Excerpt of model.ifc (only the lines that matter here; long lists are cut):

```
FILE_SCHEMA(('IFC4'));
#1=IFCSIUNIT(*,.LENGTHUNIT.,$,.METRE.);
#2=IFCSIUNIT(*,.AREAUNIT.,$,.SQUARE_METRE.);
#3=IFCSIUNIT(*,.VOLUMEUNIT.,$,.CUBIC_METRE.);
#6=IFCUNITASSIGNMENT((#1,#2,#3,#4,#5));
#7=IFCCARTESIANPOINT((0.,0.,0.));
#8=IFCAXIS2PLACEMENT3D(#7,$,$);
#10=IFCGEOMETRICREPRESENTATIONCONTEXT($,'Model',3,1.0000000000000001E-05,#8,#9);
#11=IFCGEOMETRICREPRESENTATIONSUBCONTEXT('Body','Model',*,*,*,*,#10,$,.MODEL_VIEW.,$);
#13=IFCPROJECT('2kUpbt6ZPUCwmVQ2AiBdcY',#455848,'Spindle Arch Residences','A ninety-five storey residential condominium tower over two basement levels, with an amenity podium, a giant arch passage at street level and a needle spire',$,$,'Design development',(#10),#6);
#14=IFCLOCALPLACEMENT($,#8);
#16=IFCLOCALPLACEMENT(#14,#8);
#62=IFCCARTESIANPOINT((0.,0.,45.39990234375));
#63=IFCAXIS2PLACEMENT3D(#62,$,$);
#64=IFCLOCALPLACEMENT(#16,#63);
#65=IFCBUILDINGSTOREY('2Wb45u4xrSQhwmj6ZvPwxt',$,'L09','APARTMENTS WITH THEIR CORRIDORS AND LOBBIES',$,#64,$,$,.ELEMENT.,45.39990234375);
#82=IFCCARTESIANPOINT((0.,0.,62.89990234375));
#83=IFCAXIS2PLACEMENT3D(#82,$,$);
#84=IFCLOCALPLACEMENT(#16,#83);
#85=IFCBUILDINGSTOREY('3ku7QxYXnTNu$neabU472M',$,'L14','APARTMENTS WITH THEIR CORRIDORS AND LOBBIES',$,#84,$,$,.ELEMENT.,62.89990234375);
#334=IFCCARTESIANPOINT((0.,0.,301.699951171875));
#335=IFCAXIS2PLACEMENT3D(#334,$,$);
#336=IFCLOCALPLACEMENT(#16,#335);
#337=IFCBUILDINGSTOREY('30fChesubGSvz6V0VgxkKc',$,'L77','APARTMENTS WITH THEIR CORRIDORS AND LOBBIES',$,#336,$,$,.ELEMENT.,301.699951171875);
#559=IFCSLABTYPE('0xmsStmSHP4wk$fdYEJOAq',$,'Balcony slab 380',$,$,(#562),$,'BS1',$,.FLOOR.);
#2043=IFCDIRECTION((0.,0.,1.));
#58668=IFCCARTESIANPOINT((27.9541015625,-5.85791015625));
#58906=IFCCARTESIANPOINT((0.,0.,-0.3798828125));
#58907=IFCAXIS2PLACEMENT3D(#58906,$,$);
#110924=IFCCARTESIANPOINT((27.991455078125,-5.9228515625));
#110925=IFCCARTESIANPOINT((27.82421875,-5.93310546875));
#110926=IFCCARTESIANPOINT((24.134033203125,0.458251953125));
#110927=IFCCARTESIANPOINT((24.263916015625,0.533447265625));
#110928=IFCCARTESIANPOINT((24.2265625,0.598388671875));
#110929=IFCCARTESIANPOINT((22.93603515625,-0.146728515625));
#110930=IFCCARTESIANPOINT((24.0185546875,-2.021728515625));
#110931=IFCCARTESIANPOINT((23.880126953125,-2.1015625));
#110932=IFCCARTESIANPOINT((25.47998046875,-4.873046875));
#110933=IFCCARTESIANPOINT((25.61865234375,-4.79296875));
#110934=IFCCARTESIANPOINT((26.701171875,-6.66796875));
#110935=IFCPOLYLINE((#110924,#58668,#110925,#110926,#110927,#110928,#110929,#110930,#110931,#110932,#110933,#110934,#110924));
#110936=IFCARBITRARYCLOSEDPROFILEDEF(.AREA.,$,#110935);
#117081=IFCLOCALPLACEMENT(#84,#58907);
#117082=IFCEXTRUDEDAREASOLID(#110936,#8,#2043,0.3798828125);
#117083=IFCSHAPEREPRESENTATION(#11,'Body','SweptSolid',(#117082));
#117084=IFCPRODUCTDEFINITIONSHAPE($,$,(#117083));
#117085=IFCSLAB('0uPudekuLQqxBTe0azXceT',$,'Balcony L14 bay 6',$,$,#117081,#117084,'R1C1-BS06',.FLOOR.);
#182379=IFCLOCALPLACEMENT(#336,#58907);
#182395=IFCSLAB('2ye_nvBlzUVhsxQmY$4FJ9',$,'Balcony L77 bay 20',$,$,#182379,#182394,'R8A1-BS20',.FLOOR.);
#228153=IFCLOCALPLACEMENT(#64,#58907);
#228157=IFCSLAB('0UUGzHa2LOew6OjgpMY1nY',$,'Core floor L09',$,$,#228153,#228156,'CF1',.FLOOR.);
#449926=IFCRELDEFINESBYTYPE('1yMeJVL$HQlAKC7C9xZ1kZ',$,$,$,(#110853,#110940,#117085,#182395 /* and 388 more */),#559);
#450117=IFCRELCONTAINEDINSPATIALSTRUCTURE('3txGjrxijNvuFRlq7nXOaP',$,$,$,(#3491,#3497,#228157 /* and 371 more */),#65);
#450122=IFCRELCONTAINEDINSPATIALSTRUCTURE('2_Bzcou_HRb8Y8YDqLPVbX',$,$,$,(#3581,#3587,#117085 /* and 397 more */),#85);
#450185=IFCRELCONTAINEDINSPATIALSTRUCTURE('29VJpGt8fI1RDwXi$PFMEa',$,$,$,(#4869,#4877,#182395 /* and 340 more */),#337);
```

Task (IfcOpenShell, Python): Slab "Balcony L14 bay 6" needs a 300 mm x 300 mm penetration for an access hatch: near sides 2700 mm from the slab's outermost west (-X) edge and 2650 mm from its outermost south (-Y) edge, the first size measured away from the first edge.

```python
import numpy as np
import ifcopenshell
import ifcopenshell.api.feature
import ifcopenshell.api.geometry
import ifcopenshell.api.root
import ifcopenshell.geom
import ifcopenshell.util.placement
import ifcopenshell.util.representation
import ifcopenshell.util.shape
import ifcopenshell.util.unit

model = ifcopenshell.open("model.ifc")
unit_scale = ifcopenshell.util.unit.calculate_unit_scale(model)
settings = ifcopenshell.geom.settings()


def volume(element):
    """Net volume in cubic metres, openings subtracted."""
    shape = ifcopenshell.geom.create_shape(settings, element)
    return ifcopenshell.util.shape.get_volume(shape.geometry)


slab = model.by_guid("0uPudekuLQqxBTe0azXceT")
before = volume(slab)

# Extent in the slab's own axes, in metres. The edges named are its -X and -Y sides.
slab_shape = ifcopenshell.geom.create_shape(settings, slab)
vertices = ifcopenshell.util.shape.get_vertices(slab_shape.geometry)
x_min, y_min, bottom = vertices.min(axis=0)
top = vertices[:, 2].max()

opening = ifcopenshell.api.root.create_entity(model, ifc_class="IfcOpeningElement", name="Access hatch opening", predefined_type="OPENING")
context = ifcopenshell.util.representation.get_context(model, "Model", "Body", "MODEL_VIEW")
width, depth = 0.3, 0.3
outline = [(0.0, 0.0), (width, 0.0), (width, depth), (0.0, depth), (0.0, 0.0)]
# Overshoot both faces by 50 mm so the cut is clean.
shape = ifcopenshell.api.geometry.add_slab_representation(
    model, context=context, depth=top - bottom + 0.1, polyline=outline
)
ifcopenshell.api.geometry.assign_representation(model, product=opening, representation=shape)

matrix = ifcopenshell.util.placement.get_local_placement(slab.ObjectPlacement)
matrix[:, 3] = matrix @ np.append(np.array([x_min + 2.7, y_min + 2.65, bottom - 0.05]) / unit_scale, 1.0)
ifcopenshell.api.geometry.edit_object_placement(model, product=opening, matrix=matrix, is_si=False)
ifcopenshell.api.feature.add_feature(model, feature=opening, element=slab)

after = volume(slab)

print(f"slab volume {before:.3f} -> {after:.3f} m3")

model.write("model_updated.ifc")
```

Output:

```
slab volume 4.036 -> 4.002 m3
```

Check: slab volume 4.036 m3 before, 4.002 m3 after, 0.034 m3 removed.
